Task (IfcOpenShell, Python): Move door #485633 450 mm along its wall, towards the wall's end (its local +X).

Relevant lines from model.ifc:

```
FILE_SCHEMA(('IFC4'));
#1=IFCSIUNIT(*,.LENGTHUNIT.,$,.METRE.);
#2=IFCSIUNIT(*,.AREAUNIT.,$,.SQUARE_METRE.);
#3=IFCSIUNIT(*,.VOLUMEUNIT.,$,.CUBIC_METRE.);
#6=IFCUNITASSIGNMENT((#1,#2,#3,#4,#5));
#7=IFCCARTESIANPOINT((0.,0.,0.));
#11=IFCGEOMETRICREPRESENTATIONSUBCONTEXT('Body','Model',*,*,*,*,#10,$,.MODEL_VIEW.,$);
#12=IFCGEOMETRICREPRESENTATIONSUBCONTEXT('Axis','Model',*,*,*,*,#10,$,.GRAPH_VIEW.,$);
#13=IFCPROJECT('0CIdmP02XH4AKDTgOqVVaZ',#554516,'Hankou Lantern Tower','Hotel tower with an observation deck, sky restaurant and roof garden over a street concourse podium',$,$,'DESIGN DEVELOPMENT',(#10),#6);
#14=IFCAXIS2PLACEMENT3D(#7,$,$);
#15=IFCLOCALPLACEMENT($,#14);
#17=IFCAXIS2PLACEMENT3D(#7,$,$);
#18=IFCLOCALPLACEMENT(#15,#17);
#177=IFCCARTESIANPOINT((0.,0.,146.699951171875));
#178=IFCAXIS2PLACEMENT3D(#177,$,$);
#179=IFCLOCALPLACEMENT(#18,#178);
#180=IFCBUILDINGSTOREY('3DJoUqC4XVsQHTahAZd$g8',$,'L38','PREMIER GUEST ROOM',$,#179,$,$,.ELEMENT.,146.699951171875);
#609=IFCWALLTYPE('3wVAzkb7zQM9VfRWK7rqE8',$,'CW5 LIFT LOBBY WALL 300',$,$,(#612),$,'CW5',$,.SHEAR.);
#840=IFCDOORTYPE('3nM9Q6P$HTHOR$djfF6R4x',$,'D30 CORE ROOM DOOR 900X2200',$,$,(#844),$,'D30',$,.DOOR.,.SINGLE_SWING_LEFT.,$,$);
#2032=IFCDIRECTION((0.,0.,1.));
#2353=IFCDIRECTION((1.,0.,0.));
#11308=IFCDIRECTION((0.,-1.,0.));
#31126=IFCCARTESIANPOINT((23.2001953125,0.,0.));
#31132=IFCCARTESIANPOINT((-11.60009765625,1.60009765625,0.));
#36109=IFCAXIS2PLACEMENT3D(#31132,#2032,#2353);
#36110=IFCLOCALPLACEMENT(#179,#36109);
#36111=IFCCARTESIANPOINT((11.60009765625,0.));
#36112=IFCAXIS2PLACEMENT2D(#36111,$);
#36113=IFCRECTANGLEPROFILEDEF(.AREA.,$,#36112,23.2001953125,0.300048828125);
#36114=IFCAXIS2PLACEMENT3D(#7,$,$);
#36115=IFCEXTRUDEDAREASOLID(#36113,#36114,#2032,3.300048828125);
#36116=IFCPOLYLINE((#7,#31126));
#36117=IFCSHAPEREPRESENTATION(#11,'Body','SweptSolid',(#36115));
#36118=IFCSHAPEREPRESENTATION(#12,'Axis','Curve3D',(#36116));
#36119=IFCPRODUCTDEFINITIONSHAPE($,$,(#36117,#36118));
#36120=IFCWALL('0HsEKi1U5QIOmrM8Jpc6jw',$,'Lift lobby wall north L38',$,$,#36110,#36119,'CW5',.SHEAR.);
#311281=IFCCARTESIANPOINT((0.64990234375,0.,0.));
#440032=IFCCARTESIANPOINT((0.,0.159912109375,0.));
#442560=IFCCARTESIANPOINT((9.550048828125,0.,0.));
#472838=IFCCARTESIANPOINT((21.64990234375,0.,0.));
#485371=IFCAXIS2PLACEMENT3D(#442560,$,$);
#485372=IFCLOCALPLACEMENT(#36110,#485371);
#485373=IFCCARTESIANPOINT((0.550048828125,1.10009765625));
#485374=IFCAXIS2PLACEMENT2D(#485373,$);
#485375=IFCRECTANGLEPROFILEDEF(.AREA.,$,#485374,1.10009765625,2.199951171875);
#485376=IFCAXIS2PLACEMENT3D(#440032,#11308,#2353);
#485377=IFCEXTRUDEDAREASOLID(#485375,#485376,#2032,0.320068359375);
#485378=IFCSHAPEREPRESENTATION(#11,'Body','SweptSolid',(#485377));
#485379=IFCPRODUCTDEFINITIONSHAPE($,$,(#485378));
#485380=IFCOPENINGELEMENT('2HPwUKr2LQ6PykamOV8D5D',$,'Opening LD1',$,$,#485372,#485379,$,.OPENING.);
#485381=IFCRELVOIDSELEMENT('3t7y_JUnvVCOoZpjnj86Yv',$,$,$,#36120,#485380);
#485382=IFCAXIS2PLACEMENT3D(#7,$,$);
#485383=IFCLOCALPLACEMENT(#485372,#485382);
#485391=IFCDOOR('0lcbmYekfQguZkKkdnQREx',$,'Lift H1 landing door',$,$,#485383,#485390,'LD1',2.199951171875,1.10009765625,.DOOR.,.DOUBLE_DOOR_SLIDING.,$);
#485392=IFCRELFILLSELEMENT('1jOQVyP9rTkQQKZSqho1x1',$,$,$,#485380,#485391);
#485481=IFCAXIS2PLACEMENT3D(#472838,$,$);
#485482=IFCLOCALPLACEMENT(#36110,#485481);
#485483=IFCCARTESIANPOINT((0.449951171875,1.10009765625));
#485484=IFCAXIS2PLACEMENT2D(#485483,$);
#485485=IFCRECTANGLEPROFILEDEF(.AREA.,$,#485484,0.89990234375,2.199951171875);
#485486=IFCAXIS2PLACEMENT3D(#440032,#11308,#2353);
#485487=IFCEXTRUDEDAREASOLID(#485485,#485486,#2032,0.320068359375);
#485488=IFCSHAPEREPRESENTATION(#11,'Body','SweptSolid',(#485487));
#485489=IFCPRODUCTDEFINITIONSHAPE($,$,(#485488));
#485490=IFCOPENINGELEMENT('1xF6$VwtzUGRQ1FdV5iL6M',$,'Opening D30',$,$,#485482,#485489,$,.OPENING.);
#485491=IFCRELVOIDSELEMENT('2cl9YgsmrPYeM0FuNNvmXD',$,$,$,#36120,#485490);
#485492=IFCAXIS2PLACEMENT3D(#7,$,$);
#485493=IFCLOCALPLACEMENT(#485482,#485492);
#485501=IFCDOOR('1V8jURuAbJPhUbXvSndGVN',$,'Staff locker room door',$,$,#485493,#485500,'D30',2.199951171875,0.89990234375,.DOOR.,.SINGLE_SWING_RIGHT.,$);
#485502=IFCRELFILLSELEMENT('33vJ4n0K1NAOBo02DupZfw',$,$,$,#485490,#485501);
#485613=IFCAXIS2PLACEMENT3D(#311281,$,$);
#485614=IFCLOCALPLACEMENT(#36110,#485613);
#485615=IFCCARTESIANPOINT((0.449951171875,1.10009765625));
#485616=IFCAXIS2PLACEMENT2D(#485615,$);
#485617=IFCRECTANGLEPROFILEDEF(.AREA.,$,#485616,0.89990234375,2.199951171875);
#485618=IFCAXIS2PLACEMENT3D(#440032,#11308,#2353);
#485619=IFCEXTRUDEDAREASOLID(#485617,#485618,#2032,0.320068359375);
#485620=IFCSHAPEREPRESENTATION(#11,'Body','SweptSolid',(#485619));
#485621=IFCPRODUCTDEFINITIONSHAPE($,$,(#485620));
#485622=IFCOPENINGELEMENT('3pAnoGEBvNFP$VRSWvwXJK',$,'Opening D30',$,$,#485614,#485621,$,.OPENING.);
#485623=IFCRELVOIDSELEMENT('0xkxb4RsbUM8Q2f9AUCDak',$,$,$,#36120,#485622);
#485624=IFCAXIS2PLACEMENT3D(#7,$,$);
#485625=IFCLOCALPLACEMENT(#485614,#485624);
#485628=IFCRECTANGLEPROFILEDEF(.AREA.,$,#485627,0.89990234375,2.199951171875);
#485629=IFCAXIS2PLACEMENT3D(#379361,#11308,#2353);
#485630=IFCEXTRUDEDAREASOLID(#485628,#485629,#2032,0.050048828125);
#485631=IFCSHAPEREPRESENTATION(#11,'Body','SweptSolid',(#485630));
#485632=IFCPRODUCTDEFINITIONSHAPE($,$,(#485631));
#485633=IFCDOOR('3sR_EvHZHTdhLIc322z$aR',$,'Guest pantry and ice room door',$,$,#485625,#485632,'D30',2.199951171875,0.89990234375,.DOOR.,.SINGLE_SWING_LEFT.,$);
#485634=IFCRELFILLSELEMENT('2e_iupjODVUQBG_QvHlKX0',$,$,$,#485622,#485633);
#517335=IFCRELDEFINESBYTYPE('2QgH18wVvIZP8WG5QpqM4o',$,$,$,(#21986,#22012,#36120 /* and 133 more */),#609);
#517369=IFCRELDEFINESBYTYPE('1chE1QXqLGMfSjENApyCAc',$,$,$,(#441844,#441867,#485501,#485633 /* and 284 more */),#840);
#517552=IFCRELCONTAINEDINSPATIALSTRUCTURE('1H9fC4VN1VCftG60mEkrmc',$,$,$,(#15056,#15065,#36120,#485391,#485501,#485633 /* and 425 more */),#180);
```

```python
import ifcopenshell
import ifcopenshell.api.geometry
import ifcopenshell.util.placement

model = ifcopenshell.open("model.ifc")

door = model.by_guid("3sR_EvHZHTdhLIc322z$aR")
opening = door.FillsVoids[0].RelatingOpeningElement
wall = opening.VoidsElements[0].RelatingBuildingElement

wall_matrix = ifcopenshell.util.placement.get_local_placement(wall.ObjectPlacement)
shift = wall_matrix[:3, 0] * 0.45
before = ifcopenshell.util.placement.get_local_placement(door.ObjectPlacement)[:3, 3].copy()

# The door is placed relative to its opening, so it follows when the opening moves.
matrix = ifcopenshell.util.placement.get_local_placement(opening.ObjectPlacement)
matrix[:3, 3] += shift
ifcopenshell.api.geometry.edit_object_placement(
    model, product=opening, matrix=matrix, is_si=False, should_transform_children=True
)

after = ifcopenshell.util.placement.get_local_placement(door.ObjectPlacement)[:3, 3]
print("door moved by", (after - before).round(3) + 0.0)

model.write("model_v2.ifc")
```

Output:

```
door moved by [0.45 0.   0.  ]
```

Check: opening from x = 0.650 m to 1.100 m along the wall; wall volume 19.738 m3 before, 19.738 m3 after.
